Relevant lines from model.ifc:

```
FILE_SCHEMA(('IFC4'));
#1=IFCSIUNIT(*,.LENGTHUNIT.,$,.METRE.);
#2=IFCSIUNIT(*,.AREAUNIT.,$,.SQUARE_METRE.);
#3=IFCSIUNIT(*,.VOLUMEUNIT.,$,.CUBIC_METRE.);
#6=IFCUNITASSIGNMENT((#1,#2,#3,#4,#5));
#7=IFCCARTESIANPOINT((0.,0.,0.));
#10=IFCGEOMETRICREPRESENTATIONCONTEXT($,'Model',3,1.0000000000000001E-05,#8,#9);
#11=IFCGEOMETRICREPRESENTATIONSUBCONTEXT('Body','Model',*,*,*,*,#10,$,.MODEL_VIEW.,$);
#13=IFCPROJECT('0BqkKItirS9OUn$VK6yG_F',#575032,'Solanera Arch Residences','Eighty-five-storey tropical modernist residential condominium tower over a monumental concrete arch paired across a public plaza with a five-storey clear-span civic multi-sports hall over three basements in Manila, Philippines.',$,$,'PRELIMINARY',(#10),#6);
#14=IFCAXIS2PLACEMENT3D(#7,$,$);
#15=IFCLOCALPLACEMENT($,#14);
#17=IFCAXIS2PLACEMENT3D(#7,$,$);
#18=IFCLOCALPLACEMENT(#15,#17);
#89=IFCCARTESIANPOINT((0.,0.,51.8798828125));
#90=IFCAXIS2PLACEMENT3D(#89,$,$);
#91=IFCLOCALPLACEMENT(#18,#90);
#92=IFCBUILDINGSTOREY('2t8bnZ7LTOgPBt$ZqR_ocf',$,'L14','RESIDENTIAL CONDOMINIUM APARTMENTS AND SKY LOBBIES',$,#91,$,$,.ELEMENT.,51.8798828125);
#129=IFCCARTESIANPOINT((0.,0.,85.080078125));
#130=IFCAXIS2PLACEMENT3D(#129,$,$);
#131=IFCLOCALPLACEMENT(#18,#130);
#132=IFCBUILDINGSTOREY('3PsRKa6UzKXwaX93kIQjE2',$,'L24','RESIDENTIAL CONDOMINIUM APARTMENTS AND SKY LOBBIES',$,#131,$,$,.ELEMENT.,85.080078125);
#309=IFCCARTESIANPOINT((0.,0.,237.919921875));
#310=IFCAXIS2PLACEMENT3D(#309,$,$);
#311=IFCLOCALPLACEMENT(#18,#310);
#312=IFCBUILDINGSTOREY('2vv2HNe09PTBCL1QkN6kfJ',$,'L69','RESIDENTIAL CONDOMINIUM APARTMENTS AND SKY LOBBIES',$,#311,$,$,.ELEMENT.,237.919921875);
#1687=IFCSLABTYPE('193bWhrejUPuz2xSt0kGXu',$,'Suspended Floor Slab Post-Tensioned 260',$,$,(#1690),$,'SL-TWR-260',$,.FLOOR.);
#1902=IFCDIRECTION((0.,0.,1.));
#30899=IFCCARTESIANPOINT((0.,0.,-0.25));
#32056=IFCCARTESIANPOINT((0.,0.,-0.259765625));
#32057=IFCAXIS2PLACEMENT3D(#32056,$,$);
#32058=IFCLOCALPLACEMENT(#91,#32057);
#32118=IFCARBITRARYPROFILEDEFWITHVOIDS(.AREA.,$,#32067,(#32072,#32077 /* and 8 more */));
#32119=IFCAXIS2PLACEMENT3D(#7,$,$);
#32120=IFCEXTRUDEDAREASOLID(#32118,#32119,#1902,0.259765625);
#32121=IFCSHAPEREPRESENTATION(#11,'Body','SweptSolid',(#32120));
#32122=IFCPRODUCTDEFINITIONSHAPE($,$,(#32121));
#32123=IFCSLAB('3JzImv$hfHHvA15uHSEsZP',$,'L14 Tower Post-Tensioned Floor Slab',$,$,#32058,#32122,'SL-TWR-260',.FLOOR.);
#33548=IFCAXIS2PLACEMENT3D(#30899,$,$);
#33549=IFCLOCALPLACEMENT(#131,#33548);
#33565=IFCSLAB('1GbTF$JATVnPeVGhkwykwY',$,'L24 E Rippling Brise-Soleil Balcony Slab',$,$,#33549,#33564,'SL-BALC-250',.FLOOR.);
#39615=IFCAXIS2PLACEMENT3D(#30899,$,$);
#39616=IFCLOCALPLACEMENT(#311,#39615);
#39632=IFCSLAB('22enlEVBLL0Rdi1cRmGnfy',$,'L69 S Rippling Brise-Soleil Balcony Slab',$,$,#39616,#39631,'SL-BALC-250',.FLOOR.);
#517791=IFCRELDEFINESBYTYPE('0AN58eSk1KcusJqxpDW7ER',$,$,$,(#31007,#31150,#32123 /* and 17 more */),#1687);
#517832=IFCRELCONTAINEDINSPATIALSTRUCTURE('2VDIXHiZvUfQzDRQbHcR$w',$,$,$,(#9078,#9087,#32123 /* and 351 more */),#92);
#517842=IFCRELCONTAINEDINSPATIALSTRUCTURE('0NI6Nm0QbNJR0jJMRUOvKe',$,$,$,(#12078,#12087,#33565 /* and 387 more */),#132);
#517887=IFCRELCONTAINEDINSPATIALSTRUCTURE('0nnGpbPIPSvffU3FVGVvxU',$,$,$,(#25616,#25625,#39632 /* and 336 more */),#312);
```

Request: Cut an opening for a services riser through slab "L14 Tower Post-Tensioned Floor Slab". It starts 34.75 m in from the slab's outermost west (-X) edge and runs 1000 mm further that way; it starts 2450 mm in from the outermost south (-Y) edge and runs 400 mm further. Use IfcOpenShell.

```python
import numpy as np
import ifcopenshell
import ifcopenshell.api.feature
import ifcopenshell.api.geometry
import ifcopenshell.api.root
import ifcopenshell.geom
import ifcopenshell.util.placement
import ifcopenshell.util.representation
import ifcopenshell.util.shape
import ifcopenshell.util.unit

model = ifcopenshell.open("model.ifc")
unit_scale = ifcopenshell.util.unit.calculate_unit_scale(model)
settings = ifcopenshell.geom.settings()


def volume(element):
    """Net volume in cubic metres, openings subtracted."""
    shape = ifcopenshell.geom.create_shape(settings, element)
    return ifcopenshell.util.shape.get_volume(shape.geometry)


slab = model.by_id(32123)
before = volume(slab)

# Extent in the slab's own axes, in metres. The edges named are its -X and -Y sides.
slab_shape = ifcopenshell.geom.create_shape(settings, slab)
vertices = ifcopenshell.util.shape.get_vertices(slab_shape.geometry)
x_min, y_min, bottom = vertices.min(axis=0)
top = vertices[:, 2].max()

opening = ifcopenshell.api.root.create_entity(model, ifc_class="IfcOpeningElement", name="Services riser opening", predefined_type="OPENING")
context = ifcopenshell.util.representation.get_context(model, "Model", "Body", "MODEL_VIEW")
width, depth = 1, 0.4
outline = [(0.0, 0.0), (width, 0.0), (width, depth), (0.0, depth), (0.0, 0.0)]
# Overshoot both faces by 50 mm so the cut is clean.
shape = ifcopenshell.api.geometry.add_slab_representation(
    model, context=context, depth=top - bottom + 0.1, polyline=outline
)
ifcopenshell.api.geometry.assign_representation(model, product=opening, representation=shape)

matrix = ifcopenshell.util.placement.get_local_placement(slab.ObjectPlacement)
matrix[:, 3] = matrix @ np.append(np.array([x_min + 34.75, y_min + 2.45, bottom - 0.05]) / unit_scale, 1.0)
ifcopenshell.api.geometry.edit_object_placement(model, product=opening, matrix=matrix, is_si=False)
ifcopenshell.api.feature.add_feature(model, feature=opening, element=slab)

after = volume(slab)

print(f"slab volume {before:.3f} -> {after:.3f} m3")

model.write("model_updated.ifc")
```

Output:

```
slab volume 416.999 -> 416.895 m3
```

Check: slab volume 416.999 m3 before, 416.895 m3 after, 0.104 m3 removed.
